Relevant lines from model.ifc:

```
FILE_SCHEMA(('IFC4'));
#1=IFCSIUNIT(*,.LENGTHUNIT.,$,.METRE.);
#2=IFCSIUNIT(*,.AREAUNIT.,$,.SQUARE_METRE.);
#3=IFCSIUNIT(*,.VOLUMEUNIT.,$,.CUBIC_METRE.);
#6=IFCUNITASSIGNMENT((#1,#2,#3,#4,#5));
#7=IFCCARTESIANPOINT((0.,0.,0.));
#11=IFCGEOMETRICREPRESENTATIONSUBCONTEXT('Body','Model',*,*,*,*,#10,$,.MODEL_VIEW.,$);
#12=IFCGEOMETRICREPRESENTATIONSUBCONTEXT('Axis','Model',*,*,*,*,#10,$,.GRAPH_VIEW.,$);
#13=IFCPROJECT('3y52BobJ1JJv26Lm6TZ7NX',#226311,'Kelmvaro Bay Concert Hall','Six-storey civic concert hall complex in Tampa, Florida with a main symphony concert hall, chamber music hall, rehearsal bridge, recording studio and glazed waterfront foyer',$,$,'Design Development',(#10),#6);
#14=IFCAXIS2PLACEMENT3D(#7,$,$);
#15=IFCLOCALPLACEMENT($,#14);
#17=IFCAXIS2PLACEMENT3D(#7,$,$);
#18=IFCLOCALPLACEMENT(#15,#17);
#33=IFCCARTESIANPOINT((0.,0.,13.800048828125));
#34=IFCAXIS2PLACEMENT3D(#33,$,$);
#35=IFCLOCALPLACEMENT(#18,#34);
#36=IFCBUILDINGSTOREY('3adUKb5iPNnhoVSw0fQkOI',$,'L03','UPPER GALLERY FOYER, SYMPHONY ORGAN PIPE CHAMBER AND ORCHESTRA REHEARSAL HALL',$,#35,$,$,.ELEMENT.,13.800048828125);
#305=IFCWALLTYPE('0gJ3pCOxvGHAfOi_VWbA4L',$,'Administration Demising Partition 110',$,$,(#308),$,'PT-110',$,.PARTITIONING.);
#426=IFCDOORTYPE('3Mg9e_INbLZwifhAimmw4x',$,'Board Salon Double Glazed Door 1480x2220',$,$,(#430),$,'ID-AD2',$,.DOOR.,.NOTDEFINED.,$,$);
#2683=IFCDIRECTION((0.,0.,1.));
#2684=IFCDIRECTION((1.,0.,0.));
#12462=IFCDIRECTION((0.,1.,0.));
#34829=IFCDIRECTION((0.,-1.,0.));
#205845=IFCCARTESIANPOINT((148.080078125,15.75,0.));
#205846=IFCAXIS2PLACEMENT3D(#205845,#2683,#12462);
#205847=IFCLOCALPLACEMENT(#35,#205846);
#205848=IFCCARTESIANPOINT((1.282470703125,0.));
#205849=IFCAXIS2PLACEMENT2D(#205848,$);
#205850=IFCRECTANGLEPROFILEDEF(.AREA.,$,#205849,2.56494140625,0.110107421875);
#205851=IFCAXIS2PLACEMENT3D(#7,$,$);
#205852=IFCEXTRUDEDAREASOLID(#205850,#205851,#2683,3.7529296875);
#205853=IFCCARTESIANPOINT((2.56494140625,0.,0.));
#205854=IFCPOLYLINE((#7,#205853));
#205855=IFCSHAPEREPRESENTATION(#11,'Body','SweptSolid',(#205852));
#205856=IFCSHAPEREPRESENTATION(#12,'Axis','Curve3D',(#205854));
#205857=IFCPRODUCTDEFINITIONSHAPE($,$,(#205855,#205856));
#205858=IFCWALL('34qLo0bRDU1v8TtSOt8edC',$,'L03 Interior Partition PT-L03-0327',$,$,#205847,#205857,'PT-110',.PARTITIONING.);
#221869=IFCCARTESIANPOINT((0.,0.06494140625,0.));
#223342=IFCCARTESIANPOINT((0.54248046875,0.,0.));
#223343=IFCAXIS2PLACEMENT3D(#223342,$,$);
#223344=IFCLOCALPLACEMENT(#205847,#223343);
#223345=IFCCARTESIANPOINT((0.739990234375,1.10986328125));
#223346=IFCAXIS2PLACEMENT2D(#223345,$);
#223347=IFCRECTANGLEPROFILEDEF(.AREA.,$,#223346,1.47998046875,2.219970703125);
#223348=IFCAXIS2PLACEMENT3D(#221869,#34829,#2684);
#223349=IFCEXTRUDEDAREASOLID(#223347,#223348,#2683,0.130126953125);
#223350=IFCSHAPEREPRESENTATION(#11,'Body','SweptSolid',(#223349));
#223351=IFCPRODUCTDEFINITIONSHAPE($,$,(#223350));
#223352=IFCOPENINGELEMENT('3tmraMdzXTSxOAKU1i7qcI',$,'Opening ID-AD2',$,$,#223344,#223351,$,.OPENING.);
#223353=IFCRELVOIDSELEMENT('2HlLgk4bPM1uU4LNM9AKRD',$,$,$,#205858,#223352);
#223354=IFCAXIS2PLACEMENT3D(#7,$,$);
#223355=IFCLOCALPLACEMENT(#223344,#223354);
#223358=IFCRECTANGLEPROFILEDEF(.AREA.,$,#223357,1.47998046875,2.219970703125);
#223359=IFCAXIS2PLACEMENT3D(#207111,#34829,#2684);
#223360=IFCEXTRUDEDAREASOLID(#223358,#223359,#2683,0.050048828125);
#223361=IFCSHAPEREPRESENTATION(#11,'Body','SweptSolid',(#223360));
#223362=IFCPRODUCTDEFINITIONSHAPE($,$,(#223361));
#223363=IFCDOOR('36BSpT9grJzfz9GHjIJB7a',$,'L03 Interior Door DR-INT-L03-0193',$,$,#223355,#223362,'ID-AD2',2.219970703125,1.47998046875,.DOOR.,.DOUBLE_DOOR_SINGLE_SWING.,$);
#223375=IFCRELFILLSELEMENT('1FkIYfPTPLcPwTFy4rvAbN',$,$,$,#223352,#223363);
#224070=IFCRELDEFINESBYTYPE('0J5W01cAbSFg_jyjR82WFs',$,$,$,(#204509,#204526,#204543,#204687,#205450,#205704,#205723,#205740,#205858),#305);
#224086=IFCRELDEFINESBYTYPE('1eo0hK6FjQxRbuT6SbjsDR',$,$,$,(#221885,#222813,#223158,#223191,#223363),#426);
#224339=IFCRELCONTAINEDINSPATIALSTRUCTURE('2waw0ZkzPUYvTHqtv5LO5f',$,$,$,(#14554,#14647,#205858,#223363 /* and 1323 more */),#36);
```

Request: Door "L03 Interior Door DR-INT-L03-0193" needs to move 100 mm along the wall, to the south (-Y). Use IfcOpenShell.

```python
import ifcopenshell
import ifcopenshell.api.geometry
import ifcopenshell.util.placement
import ifcopenshell.util.unit

model = ifcopenshell.open("model.ifc")
unit_scale = ifcopenshell.util.unit.calculate_unit_scale(model)

door = model.by_id(223363)
opening = door.FillsVoids[0].RelatingOpeningElement
wall = opening.VoidsElements[0].RelatingBuildingElement

wall_matrix = ifcopenshell.util.placement.get_local_placement(wall.ObjectPlacement)
shift = wall_matrix[:3, 0] * -0.1 / unit_scale
before = ifcopenshell.util.placement.get_local_placement(door.ObjectPlacement)[:3, 3].copy()

# The door is placed relative to its opening, so it follows when the opening moves.
matrix = ifcopenshell.util.placement.get_local_placement(opening.ObjectPlacement)
matrix[:3, 3] += shift
ifcopenshell.api.geometry.edit_object_placement(
    model, product=opening, matrix=matrix, is_si=False, should_transform_children=True
)

after = ifcopenshell.util.placement.get_local_placement(door.ObjectPlacement)[:3, 3]
print("door moved by", (after - before).round(3) + 0.0)

model.write("model_updated.ifc")
```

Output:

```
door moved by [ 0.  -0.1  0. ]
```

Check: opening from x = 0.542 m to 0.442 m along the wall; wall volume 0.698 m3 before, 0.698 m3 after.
